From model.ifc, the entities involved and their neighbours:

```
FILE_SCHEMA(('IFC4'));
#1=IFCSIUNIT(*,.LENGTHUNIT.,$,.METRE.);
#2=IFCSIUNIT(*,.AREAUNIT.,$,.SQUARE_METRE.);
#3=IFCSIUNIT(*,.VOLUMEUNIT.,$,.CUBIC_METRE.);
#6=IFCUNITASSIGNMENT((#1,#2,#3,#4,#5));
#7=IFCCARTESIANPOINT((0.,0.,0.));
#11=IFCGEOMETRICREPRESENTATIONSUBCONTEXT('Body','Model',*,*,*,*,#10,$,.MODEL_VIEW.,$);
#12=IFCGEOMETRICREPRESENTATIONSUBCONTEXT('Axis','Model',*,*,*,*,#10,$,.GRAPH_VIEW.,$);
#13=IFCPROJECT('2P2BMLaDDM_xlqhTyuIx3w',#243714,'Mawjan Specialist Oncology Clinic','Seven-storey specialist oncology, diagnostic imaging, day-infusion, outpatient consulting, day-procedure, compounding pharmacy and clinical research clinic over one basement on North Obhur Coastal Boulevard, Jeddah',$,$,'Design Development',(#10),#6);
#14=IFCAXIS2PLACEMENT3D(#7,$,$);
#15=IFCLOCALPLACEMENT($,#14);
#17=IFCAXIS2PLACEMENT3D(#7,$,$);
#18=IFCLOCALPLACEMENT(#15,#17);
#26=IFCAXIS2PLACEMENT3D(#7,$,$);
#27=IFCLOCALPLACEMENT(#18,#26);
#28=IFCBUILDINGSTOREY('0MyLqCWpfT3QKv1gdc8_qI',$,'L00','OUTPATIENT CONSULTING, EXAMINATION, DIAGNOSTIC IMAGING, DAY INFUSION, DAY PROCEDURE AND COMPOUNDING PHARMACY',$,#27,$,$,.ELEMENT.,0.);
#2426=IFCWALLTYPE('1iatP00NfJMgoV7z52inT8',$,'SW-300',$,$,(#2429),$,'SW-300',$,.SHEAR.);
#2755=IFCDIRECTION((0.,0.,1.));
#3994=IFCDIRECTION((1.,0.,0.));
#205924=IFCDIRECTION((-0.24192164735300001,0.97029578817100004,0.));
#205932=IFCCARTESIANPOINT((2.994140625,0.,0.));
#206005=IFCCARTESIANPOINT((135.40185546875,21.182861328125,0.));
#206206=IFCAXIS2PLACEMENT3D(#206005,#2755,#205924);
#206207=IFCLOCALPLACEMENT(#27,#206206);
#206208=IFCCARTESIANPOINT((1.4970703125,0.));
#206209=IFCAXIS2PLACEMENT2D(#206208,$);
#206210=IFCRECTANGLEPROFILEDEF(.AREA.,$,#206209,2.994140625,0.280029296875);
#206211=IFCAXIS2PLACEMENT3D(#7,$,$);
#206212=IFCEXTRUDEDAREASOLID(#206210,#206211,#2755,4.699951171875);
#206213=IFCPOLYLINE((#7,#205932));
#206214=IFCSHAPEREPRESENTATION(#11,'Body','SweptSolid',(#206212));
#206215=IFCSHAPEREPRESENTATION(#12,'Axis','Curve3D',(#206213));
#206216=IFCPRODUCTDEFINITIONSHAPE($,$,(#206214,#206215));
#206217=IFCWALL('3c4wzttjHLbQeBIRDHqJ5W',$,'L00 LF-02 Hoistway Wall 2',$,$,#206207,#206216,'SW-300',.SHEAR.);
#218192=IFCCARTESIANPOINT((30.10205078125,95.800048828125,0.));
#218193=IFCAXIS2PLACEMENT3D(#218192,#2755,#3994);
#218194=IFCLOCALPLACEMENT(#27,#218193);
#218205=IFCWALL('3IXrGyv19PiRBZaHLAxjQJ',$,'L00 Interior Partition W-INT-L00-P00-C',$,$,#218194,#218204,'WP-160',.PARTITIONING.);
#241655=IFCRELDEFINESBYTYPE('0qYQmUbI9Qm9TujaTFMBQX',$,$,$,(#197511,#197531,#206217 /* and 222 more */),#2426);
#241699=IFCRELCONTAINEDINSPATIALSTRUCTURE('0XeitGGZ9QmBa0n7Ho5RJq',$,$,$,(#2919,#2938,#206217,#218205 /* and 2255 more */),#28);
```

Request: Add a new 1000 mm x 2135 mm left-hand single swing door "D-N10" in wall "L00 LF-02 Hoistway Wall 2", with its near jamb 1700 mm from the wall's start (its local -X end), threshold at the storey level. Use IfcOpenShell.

```python
import numpy as np
import ifcopenshell
import ifcopenshell.api.feature
import ifcopenshell.api.geometry
import ifcopenshell.api.root
import ifcopenshell.api.spatial
import ifcopenshell.geom
import ifcopenshell.util.element
import ifcopenshell.util.placement
import ifcopenshell.util.representation
import ifcopenshell.util.shape
import ifcopenshell.util.unit

model = ifcopenshell.open("model.ifc")
unit_scale = ifcopenshell.util.unit.calculate_unit_scale(model)
settings = ifcopenshell.geom.settings()


def volume(element):
    """Net volume in cubic metres, openings subtracted."""
    shape = ifcopenshell.geom.create_shape(settings, element)
    return ifcopenshell.util.shape.get_volume(shape.geometry)


wall = model.by_guid("3c4wzttjHLbQeBIRDHqJ5W")
storey = ifcopenshell.util.element.get_container(wall, ifc_class="IfcBuildingStorey")
context = ifcopenshell.util.representation.get_context(model, "Model", "Body", "MODEL_VIEW")
before = volume(wall)

width, height, from_end, sill = 1, 2.135, 1.7, 0.0  # metres

# The wall runs along its own X axis, and the end named is its -X end.
wall_shape = ifcopenshell.geom.create_shape(settings, wall)
x, y, z = ifcopenshell.util.shape.get_vertices(wall_shape.geometry).T
start = x.min() + from_end
face, thickness = float(y.min()), float(y.max() - y.min())
wall_matrix = ifcopenshell.util.placement.get_local_placement(wall.ObjectPlacement)
level = ifcopenshell.util.placement.get_local_placement(storey.ObjectPlacement)[2, 3]


def in_wall(x, y):
    """Placement at x, y metres in the wall's axes, at sill height."""
    matrix = wall_matrix.copy()
    matrix[:, 3] = wall_matrix @ np.array([x / unit_scale, y / unit_scale, 0.0, 1.0])
    matrix[2, 3] = level + sill / unit_scale
    return matrix


# Opening: a box that overshoots both wall faces by 50 mm.
opening = ifcopenshell.api.root.create_entity(model, ifc_class="IfcOpeningElement", predefined_type="OPENING")
box = ifcopenshell.api.geometry.add_wall_representation(
    model, context=context, length=width, height=height, thickness=thickness + 0.1
)
ifcopenshell.api.geometry.assign_representation(model, product=opening, representation=box)
ifcopenshell.api.geometry.edit_object_placement(model, product=opening, matrix=in_wall(start, face - 0.05), is_si=False)
ifcopenshell.api.feature.add_feature(model, feature=opening, element=wall)

door = ifcopenshell.api.root.create_entity(model, ifc_class="IfcDoor", name="D-N10", predefined_type="DOOR")
door.OverallWidth, door.OverallHeight = width / unit_scale, height / unit_scale
door.OperationType = "SINGLE_SWING_LEFT"
body = ifcopenshell.api.geometry.add_door_representation(
    model,
    context=context,
    overall_width=door.OverallWidth,
    overall_height=door.OverallHeight,
    operation_type="SINGLE_SWING_LEFT",
    lining_properties={"LiningDepth": thickness / unit_scale, "ThresholdDepth": thickness / unit_scale},
)
ifcopenshell.api.geometry.assign_representation(model, product=door, representation=body)
ifcopenshell.api.spatial.assign_container(model, products=[door], relating_structure=storey)
ifcopenshell.api.feature.add_filling(model, opening=opening, element=door)

# The lining spans the wall, so the door starts at the wall face.
ifcopenshell.api.geometry.edit_object_placement(model, product=door, matrix=in_wall(start, face), is_si=False)

after = volume(wall)

print(f"wall volume {before:.3f} -> {after:.3f} m3")

model.write("model_edited.ifc")
```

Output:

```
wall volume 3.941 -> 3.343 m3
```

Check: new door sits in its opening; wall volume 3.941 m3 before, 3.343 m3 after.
